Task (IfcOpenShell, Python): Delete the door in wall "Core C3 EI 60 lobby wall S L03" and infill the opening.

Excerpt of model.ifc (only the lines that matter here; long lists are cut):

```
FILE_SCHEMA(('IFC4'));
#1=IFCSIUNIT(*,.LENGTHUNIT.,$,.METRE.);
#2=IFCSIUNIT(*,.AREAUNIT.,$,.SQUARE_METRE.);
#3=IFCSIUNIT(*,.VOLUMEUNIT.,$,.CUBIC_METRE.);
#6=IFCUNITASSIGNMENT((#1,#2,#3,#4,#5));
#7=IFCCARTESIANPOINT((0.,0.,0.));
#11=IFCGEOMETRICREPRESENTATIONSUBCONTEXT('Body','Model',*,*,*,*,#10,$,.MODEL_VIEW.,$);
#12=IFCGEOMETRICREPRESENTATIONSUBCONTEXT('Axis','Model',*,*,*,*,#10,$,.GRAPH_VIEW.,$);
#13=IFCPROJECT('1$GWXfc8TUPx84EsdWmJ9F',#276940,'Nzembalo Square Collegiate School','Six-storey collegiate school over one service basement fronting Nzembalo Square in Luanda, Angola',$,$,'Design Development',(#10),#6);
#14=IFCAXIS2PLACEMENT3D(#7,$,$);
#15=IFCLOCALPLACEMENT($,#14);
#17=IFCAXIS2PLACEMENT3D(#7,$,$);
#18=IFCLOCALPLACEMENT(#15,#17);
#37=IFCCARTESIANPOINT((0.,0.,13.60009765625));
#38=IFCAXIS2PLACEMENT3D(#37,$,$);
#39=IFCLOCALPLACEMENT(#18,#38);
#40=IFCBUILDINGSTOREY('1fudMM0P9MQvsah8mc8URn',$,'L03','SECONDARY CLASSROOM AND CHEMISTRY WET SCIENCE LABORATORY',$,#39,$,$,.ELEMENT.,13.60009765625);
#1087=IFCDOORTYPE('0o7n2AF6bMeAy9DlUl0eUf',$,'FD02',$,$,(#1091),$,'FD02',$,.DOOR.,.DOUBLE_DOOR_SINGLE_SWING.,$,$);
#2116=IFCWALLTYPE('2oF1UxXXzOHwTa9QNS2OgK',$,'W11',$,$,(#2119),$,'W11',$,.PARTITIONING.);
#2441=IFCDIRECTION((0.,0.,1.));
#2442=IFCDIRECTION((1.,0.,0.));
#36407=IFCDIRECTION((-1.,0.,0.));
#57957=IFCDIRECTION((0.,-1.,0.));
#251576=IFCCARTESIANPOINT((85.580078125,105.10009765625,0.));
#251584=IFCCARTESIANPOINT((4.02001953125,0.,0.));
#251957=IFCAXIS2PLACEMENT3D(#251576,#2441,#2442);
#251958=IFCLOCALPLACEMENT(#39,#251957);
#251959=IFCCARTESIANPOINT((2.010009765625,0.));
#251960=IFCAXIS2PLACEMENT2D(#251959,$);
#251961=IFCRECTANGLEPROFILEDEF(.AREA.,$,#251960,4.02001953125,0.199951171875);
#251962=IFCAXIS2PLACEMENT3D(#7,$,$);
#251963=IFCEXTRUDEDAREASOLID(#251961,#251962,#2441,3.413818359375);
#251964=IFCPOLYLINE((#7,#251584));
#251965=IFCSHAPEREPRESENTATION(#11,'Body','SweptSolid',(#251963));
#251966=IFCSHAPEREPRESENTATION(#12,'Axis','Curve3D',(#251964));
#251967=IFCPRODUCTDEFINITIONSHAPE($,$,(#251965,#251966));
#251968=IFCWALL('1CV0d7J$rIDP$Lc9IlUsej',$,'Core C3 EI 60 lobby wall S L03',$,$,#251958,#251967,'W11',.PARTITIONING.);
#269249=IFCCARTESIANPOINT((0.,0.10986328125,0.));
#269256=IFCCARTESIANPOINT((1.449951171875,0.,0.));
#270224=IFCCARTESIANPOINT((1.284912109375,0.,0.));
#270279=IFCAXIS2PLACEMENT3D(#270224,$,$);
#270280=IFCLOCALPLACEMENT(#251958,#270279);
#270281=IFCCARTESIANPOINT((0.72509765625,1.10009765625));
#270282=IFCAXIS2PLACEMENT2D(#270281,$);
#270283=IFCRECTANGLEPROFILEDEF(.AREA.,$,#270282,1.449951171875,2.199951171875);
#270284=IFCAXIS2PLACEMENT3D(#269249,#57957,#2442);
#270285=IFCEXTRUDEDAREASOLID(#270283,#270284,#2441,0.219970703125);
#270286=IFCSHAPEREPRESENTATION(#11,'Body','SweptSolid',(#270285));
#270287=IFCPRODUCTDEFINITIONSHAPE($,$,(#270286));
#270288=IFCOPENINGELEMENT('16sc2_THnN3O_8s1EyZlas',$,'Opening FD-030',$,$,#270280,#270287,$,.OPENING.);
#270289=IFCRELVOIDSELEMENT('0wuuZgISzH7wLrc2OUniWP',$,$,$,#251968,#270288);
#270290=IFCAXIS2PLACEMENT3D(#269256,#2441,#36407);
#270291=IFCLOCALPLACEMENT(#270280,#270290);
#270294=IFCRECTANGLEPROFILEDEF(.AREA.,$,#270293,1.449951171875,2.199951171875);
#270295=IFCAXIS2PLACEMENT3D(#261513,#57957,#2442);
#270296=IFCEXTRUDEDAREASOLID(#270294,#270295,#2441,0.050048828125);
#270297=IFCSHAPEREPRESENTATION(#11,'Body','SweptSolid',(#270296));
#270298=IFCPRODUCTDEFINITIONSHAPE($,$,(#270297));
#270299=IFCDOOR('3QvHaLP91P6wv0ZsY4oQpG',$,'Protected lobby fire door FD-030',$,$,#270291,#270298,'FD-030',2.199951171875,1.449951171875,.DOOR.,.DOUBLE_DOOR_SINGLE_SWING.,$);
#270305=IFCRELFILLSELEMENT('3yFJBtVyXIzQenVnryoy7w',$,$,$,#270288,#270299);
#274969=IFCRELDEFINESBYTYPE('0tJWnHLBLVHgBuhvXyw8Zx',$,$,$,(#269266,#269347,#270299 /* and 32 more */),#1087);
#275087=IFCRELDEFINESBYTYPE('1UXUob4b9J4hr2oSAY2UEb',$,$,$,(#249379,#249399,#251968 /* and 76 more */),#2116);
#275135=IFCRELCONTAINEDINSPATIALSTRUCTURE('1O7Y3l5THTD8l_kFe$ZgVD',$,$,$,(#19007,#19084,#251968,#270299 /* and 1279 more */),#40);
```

```python
import ifcopenshell
import ifcopenshell.api.feature
import ifcopenshell.api.root
import ifcopenshell.geom
import ifcopenshell.util.shape

model = ifcopenshell.open("model.ifc")
settings = ifcopenshell.geom.settings()


def volume(element):
    """Net volume in cubic metres, openings subtracted."""
    shape = ifcopenshell.geom.create_shape(settings, element)
    return ifcopenshell.util.shape.get_volume(shape.geometry)


door = model.by_id(270299)
opening = door.FillsVoids[0].RelatingOpeningElement
wall = opening.VoidsElements[0].RelatingBuildingElement
before = volume(wall)

ifcopenshell.api.root.remove_product(model, product=door)
ifcopenshell.api.feature.remove_feature(model, feature=opening)

after = volume(wall)

print(f"wall volume {before:.3f} -> {after:.3f} m3")

model.write("model_edited.ifc")
```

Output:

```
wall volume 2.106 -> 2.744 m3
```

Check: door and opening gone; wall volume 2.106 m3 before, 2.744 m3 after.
